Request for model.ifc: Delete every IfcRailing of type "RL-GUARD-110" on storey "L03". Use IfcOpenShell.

First a look at what the model holds.

```python
import ifcopenshell
import ifcopenshell.util.element

model = ifcopenshell.open("model.ifc")
print(model.schema)
storey = next(s for s in model.by_type("IfcBuildingStorey") if s.Name == "L03")
railings = [e for e in ifcopenshell.util.element.get_decomposition(storey) if e.is_a("IfcRailing")]
seen = {}
for e in railings:
    element_type = ifcopenshell.util.element.get_type(e)
    name = element_type.Name if element_type not in (None, e) else None
    seen[name] = seen.get(name, 0) + 1
for name, count in sorted(seen.items(), key=str):
    print(count, "x", name)
```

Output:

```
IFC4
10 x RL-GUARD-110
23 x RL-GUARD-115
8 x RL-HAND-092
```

```python
import ifcopenshell
import ifcopenshell.api.root
import ifcopenshell.util.element

model = ifcopenshell.open("model.ifc")

storey = next(s for s in model.by_type("IfcBuildingStorey") if s.Name == "L03")
railings = [e for e in ifcopenshell.util.element.get_decomposition(storey) if e.is_a("IfcRailing")]
targets = [e for e in railings if (t := ifcopenshell.util.element.get_type(e)) not in (None, e) and t.Name == "RL-GUARD-110"]

for e in targets:
    ifcopenshell.api.root.remove_product(model, product=e)
print(len(targets), "removed")

model.write("model_rev.ifc")
```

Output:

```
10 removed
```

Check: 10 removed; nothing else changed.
